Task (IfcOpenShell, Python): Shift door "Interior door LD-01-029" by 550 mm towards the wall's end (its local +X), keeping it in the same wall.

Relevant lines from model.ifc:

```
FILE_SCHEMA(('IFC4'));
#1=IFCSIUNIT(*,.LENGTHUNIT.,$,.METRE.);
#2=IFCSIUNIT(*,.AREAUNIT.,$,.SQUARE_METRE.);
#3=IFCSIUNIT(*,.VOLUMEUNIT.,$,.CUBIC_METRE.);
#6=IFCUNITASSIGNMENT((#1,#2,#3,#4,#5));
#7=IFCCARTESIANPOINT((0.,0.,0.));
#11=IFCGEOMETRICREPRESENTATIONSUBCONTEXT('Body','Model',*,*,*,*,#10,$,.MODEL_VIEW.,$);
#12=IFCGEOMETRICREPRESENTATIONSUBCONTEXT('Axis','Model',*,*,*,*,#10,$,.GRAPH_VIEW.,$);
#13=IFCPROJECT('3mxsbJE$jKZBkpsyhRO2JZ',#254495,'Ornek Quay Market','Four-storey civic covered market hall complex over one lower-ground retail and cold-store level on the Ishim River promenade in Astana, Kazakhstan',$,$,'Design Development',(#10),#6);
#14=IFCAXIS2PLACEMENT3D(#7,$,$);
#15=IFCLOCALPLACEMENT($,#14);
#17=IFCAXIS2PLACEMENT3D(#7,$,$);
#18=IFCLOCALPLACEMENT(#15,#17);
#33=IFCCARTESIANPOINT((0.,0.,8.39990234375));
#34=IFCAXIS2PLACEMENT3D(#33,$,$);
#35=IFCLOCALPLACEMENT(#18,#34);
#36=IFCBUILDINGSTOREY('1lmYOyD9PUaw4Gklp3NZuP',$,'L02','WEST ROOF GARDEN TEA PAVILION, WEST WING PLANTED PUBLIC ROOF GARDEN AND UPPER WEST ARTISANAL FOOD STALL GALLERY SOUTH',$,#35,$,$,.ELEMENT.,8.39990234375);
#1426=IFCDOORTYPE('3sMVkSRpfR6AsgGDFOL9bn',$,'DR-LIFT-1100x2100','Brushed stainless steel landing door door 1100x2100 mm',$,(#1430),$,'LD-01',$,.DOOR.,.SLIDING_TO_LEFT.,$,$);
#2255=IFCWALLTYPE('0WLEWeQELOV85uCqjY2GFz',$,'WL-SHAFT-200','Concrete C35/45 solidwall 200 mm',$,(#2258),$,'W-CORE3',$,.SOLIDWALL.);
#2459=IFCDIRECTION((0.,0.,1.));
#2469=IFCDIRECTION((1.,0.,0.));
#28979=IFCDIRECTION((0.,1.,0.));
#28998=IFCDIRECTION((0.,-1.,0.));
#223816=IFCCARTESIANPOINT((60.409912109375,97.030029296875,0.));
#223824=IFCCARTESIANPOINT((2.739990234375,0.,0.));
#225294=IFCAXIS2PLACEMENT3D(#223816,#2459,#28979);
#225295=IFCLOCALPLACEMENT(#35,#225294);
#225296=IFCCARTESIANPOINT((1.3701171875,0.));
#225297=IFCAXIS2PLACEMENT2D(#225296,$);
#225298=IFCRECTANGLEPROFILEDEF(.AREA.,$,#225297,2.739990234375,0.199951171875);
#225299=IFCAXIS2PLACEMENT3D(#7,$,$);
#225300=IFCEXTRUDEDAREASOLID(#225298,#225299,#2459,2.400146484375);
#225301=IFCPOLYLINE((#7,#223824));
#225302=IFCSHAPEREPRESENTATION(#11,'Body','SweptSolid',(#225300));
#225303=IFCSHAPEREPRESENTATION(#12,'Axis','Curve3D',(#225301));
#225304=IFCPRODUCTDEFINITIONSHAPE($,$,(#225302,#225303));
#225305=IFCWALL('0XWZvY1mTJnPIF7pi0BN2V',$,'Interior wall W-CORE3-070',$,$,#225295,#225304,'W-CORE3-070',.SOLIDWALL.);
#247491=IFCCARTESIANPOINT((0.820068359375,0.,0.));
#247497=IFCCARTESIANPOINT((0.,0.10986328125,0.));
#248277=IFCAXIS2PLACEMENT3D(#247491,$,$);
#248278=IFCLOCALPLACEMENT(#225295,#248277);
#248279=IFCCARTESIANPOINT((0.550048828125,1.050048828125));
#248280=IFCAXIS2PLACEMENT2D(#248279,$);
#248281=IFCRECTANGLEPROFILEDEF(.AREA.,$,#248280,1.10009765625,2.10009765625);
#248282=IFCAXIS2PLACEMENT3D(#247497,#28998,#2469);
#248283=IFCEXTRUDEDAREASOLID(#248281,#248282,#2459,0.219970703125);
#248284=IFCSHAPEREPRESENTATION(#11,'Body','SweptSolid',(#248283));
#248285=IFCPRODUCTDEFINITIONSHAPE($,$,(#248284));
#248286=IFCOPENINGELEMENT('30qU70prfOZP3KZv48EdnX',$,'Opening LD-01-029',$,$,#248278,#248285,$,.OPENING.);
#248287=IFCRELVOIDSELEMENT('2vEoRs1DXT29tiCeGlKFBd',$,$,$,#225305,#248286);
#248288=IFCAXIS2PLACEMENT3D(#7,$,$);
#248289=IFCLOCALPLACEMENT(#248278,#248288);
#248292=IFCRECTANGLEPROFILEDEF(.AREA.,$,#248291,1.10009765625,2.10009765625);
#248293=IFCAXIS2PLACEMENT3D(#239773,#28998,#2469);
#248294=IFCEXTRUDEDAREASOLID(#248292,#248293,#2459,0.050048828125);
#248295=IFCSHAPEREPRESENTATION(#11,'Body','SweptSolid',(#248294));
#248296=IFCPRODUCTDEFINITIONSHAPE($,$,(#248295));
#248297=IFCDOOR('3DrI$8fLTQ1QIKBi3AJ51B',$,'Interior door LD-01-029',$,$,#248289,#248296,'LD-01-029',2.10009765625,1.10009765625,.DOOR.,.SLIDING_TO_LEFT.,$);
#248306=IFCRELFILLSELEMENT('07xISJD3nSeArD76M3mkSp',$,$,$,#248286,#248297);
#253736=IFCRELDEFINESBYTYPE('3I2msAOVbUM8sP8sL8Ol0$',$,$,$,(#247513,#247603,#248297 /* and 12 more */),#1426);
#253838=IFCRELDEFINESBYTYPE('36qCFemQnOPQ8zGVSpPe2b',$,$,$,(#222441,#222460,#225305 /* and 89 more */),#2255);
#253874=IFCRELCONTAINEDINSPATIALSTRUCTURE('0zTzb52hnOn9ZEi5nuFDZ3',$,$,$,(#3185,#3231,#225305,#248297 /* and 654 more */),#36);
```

```python
import ifcopenshell
import ifcopenshell.api.geometry
import ifcopenshell.util.placement

model = ifcopenshell.open("model.ifc")

door = model.by_guid("3DrI$8fLTQ1QIKBi3AJ51B")
opening = door.FillsVoids[0].RelatingOpeningElement
wall = opening.VoidsElements[0].RelatingBuildingElement

wall_matrix = ifcopenshell.util.placement.get_local_placement(wall.ObjectPlacement)
shift = wall_matrix[:3, 0] * 0.55
before = ifcopenshell.util.placement.get_local_placement(door.ObjectPlacement)[:3, 3].copy()

# The door is placed relative to its opening, so it follows when the opening moves.
matrix = ifcopenshell.util.placement.get_local_placement(opening.ObjectPlacement)
matrix[:3, 3] += shift
ifcopenshell.api.geometry.edit_object_placement(
    model, product=opening, matrix=matrix, is_si=False, should_transform_children=True
)

after = ifcopenshell.util.placement.get_local_placement(door.ObjectPlacement)[:3, 3]
print("door moved by", (after - before).round(3) + 0.0)

model.write("model_rev.ifc")
```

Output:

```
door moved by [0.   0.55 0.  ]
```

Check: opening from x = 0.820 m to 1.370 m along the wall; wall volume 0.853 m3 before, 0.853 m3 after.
